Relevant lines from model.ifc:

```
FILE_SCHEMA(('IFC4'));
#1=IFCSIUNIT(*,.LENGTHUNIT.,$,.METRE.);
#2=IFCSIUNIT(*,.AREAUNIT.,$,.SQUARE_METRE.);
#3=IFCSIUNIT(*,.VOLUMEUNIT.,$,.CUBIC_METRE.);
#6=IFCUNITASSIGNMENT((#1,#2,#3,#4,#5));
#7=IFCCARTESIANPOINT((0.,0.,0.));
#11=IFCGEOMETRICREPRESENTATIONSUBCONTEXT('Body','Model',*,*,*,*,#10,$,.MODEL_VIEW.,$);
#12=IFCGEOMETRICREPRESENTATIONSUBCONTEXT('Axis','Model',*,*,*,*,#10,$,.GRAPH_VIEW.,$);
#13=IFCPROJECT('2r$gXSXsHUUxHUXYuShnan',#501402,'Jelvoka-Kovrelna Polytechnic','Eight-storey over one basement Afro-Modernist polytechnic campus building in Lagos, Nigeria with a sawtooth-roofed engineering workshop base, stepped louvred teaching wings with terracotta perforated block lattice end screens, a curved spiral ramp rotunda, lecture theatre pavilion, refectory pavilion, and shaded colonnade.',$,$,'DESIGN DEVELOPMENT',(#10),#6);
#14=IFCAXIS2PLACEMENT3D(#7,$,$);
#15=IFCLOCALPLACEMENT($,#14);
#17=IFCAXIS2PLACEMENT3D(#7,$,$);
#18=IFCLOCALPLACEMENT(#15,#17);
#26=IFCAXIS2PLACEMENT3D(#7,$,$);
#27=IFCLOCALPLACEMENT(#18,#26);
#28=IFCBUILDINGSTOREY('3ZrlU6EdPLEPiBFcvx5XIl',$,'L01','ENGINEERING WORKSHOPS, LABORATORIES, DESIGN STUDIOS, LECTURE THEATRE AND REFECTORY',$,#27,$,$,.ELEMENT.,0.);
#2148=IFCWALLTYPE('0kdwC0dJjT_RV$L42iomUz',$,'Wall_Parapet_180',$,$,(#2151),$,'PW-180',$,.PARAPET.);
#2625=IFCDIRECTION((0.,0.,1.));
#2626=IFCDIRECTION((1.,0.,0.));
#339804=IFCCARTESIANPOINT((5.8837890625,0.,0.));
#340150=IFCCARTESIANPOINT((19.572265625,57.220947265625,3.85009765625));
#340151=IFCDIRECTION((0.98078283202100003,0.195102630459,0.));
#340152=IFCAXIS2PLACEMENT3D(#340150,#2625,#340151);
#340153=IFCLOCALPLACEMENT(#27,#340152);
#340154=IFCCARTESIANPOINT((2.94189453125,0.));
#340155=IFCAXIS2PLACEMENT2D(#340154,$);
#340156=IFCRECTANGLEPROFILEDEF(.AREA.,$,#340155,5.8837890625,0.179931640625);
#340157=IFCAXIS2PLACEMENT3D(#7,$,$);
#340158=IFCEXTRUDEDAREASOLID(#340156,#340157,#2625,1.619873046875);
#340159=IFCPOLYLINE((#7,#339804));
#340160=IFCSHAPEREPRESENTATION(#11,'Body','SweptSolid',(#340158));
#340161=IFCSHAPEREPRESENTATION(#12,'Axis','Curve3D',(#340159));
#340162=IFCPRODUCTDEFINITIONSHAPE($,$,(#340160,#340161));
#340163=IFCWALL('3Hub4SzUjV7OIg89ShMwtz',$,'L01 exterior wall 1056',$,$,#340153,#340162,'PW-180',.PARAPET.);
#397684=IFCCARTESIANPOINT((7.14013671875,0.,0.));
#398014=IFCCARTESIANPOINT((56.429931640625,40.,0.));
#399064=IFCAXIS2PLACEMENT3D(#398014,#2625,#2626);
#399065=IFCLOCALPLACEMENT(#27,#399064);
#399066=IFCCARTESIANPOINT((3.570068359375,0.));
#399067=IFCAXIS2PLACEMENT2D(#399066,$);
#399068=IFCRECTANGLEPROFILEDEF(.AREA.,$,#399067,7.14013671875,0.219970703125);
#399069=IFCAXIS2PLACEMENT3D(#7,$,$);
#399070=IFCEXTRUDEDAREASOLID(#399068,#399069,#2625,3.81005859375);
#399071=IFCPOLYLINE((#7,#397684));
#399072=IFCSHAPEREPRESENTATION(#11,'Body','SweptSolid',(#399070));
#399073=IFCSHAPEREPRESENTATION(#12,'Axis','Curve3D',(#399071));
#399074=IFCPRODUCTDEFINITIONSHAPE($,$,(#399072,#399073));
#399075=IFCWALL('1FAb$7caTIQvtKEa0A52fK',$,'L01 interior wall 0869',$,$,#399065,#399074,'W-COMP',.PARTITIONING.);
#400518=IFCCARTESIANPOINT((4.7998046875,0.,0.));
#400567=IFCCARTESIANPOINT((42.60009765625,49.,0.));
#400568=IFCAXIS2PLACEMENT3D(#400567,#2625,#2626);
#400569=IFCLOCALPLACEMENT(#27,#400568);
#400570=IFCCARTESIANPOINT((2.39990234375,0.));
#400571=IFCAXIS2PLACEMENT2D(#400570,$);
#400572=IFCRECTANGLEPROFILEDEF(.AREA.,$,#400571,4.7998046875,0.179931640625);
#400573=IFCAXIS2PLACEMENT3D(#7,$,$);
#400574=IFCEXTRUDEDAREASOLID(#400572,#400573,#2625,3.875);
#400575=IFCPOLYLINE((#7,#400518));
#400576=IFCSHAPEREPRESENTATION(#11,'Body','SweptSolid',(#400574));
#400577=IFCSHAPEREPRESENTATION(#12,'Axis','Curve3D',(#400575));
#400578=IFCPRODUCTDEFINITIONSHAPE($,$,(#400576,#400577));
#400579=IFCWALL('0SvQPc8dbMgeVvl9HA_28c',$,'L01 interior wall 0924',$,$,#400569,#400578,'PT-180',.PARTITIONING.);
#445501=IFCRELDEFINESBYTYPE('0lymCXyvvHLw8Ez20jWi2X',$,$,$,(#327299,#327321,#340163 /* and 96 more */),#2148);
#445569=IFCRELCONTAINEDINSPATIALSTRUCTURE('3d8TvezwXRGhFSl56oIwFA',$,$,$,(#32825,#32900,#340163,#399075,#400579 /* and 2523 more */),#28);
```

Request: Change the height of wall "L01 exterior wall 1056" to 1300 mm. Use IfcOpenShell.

```python
import ifcopenshell
import ifcopenshell.geom
import ifcopenshell.util.representation
import ifcopenshell.util.shape

model = ifcopenshell.open("model.ifc")
settings = ifcopenshell.geom.settings()


def volume(element):
    """Net volume in cubic metres, openings subtracted."""
    shape = ifcopenshell.geom.create_shape(settings, element)
    return ifcopenshell.util.shape.get_volume(shape.geometry)


wall = model.by_id(340163)
before = volume(wall)

body = ifcopenshell.util.representation.get_representation(wall, "Model", "Body")
solid = body.Items[0]
old_height = solid.Depth
solid.Depth = 1.3
after = volume(wall)

print(f"height {old_height:g} -> {solid.Depth:g}, volume {before:.3f} -> {after:.3f} m3")

model.write("model_rev.ifc")
```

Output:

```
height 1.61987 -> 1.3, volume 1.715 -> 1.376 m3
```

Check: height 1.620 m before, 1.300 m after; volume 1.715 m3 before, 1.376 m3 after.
